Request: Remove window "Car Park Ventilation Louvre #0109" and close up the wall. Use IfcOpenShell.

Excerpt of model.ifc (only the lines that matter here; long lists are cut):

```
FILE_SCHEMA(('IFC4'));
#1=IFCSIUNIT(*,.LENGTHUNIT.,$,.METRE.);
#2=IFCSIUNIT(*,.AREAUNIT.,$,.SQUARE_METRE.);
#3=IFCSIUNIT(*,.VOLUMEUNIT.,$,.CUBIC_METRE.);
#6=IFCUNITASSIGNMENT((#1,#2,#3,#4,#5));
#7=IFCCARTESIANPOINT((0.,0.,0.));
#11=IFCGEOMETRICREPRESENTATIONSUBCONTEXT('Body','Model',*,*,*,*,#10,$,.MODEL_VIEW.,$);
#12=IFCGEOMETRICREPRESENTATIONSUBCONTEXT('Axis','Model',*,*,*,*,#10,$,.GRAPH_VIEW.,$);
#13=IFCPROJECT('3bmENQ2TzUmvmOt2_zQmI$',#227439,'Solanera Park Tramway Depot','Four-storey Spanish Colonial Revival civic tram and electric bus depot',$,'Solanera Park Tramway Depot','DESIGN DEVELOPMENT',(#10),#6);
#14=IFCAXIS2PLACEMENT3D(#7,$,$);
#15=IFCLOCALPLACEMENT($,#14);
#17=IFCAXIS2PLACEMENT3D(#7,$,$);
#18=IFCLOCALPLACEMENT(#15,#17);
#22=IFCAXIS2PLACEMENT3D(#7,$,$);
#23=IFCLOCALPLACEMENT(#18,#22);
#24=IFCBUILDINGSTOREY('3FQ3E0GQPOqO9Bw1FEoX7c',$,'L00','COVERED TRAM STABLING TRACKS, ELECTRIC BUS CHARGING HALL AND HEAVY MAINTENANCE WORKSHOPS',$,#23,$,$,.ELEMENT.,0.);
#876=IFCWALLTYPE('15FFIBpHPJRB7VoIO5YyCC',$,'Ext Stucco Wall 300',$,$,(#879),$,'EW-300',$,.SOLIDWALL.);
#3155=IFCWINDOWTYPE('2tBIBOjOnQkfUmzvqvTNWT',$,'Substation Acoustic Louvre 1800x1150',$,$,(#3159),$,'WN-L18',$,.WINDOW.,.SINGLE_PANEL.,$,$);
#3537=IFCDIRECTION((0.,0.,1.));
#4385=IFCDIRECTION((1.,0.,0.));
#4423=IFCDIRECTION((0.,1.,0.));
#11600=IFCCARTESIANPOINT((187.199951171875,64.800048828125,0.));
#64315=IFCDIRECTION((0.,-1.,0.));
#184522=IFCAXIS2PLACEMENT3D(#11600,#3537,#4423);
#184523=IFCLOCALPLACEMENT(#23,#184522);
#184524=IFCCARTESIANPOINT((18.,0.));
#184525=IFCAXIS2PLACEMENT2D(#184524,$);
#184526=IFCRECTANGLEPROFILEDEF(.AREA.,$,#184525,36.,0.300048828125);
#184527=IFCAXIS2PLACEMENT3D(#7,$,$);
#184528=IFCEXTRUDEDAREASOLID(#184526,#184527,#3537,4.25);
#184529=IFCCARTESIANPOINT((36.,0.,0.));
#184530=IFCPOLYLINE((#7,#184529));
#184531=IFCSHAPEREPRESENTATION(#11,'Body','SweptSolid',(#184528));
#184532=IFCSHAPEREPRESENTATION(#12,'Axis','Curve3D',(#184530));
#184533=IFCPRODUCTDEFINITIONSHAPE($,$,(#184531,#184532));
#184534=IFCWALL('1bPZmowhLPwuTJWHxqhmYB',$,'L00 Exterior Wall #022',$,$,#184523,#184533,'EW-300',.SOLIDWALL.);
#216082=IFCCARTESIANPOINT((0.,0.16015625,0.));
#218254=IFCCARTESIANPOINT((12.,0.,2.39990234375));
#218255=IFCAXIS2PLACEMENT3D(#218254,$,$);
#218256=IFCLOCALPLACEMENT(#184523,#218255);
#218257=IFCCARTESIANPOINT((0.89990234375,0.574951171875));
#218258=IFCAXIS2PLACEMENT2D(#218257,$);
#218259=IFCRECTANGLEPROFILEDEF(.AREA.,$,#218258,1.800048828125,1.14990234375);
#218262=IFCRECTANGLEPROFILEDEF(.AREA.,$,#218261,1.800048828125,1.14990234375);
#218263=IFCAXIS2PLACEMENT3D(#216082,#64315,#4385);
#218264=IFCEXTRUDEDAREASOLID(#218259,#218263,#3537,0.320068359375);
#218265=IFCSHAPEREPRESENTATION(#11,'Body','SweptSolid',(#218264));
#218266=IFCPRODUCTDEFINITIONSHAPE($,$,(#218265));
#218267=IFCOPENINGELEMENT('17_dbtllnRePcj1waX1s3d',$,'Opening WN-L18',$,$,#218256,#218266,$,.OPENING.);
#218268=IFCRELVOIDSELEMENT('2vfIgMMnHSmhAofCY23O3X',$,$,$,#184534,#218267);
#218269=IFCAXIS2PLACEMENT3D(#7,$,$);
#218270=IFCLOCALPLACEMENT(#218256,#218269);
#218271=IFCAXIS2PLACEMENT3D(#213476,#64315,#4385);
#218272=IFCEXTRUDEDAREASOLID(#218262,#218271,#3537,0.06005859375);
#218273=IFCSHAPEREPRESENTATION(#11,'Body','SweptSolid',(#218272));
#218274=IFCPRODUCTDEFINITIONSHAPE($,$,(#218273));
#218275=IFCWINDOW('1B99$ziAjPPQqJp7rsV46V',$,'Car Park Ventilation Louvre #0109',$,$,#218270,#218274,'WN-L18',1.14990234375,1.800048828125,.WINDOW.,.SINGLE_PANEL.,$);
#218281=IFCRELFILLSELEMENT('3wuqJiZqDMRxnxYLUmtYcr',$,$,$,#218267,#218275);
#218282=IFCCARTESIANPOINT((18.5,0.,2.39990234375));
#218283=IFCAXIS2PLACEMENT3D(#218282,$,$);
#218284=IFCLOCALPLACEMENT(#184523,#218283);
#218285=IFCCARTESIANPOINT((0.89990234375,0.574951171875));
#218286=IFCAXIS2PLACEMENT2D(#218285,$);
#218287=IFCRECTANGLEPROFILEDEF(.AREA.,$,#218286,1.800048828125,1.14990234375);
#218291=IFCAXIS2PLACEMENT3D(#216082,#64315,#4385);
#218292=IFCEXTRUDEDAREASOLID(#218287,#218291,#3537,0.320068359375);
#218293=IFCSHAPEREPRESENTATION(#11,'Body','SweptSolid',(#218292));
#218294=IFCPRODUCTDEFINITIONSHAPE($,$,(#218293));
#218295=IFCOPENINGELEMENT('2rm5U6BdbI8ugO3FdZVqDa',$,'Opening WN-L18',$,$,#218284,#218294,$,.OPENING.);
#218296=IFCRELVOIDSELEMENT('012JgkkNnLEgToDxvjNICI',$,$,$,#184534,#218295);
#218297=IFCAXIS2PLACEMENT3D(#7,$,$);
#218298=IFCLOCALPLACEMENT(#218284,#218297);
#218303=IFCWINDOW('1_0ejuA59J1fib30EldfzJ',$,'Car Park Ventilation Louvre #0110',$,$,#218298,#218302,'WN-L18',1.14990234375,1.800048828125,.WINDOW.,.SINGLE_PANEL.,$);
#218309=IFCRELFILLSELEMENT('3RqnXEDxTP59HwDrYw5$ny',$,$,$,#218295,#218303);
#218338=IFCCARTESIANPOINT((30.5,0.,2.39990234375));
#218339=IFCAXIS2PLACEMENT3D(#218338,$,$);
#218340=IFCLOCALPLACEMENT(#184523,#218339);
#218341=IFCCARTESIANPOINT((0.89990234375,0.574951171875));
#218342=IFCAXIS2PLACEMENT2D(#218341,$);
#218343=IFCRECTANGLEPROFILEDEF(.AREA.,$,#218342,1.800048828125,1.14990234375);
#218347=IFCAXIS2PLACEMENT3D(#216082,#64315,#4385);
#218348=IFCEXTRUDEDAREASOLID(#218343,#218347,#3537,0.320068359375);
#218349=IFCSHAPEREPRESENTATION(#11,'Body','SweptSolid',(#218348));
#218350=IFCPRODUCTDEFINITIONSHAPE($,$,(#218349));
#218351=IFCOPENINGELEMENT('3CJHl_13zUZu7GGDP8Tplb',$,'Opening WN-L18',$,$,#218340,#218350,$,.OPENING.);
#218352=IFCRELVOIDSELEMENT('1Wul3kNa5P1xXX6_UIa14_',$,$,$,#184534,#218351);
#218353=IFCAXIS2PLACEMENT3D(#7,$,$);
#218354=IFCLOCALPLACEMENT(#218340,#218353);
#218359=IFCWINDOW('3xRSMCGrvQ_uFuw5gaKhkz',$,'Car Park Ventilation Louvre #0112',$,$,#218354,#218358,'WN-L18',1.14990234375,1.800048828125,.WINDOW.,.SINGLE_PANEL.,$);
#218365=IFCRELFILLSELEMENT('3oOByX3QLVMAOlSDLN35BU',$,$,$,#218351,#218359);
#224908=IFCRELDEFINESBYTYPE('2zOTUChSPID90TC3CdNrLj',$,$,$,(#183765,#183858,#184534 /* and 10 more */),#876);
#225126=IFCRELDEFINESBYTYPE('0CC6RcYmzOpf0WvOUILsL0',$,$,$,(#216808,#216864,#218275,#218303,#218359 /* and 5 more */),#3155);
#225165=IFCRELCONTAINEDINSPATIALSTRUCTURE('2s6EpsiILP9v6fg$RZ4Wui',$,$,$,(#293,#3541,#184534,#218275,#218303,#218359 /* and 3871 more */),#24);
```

```python
import ifcopenshell
import ifcopenshell.api.feature
import ifcopenshell.api.root
import ifcopenshell.geom
import ifcopenshell.util.shape

model = ifcopenshell.open("model.ifc")
settings = ifcopenshell.geom.settings()


def volume(element):
    """Net volume in cubic metres, openings subtracted."""
    shape = ifcopenshell.geom.create_shape(settings, element)
    return ifcopenshell.util.shape.get_volume(shape.geometry)


window = model.by_guid("1B99$ziAjPPQqJp7rsV46V")
opening = window.FillsVoids[0].RelatingOpeningElement
wall = opening.VoidsElements[0].RelatingBuildingElement
before = volume(wall)

ifcopenshell.api.root.remove_product(model, product=window)
ifcopenshell.api.feature.remove_feature(model, feature=opening)

after = volume(wall)

print(f"wall volume {before:.3f} -> {after:.3f} m3")

model.write("model_edited.ifc")
```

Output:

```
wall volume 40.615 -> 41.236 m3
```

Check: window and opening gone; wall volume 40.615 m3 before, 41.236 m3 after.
